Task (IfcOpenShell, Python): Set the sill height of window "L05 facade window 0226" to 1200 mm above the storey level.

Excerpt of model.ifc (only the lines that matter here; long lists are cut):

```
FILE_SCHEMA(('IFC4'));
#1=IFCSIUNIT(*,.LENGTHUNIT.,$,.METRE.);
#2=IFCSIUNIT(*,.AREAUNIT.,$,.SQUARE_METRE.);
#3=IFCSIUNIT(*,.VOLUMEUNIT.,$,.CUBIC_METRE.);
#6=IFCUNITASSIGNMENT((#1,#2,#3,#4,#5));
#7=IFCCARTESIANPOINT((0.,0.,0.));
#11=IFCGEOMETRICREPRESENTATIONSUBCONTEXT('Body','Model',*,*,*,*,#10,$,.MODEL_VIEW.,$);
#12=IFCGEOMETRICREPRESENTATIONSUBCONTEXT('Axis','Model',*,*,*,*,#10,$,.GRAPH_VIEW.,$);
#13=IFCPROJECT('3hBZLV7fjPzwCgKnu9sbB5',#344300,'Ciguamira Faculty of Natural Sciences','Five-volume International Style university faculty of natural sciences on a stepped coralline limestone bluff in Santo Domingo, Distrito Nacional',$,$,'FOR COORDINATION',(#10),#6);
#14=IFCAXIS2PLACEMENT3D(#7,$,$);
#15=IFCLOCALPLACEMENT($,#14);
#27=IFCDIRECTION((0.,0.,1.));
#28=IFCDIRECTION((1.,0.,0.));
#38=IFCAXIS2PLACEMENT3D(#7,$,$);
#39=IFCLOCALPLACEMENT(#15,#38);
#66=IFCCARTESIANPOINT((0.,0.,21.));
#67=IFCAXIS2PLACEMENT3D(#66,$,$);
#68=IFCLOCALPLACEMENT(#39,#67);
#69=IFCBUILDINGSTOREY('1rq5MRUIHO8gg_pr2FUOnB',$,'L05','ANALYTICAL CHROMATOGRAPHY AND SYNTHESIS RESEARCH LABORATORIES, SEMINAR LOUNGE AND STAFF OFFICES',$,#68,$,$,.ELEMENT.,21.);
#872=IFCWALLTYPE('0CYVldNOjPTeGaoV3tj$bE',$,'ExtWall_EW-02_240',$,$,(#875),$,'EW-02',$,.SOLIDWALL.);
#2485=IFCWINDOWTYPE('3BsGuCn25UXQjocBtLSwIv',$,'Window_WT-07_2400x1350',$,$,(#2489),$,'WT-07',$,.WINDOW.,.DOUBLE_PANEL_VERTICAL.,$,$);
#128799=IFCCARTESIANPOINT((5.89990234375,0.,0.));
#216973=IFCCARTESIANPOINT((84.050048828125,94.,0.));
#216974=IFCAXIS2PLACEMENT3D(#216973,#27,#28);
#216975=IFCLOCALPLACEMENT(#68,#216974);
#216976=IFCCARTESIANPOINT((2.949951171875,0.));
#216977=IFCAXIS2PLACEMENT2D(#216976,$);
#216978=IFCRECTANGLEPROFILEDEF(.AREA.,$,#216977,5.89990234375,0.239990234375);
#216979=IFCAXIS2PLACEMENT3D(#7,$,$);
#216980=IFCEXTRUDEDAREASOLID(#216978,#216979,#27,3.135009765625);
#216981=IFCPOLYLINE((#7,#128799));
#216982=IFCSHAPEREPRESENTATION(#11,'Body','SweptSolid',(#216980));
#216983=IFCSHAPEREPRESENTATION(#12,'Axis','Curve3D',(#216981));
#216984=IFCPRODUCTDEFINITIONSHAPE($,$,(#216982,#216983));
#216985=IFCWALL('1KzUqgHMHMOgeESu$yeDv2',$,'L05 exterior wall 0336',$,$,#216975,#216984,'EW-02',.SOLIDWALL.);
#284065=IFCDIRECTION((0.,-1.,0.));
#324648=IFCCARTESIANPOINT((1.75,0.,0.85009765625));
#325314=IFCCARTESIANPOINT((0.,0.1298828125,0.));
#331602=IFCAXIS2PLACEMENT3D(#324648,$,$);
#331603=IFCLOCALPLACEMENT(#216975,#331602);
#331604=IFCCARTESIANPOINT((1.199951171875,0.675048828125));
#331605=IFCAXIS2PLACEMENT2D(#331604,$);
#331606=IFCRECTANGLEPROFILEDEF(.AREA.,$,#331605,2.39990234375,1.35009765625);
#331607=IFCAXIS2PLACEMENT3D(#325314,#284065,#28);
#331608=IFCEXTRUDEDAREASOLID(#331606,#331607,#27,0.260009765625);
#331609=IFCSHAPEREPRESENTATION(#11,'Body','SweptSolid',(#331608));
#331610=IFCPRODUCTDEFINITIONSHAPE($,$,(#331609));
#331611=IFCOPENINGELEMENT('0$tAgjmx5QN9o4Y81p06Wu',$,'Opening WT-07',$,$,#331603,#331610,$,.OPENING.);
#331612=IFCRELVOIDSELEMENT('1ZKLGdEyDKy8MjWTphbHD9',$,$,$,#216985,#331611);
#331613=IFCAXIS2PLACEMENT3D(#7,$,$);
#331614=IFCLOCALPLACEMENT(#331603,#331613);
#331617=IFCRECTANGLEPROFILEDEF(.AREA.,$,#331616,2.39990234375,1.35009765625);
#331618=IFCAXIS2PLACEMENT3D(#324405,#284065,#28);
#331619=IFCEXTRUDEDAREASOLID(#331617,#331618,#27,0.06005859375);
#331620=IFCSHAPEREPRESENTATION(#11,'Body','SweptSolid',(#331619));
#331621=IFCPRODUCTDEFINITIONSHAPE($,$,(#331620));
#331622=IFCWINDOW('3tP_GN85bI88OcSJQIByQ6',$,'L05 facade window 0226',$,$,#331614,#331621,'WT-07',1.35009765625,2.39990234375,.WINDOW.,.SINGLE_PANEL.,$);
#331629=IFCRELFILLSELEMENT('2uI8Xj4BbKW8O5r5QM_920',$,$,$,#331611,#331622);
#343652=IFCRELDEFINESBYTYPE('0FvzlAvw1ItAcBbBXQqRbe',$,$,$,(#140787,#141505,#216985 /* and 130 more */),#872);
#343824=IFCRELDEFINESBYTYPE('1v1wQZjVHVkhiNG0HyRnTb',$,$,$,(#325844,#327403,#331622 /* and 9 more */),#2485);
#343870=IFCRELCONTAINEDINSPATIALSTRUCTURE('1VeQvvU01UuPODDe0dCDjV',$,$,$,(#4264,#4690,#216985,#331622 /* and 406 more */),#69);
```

```python
import numpy as np
import ifcopenshell
import ifcopenshell.api.geometry
import ifcopenshell.geom
import ifcopenshell.util.element
import ifcopenshell.util.placement
import ifcopenshell.util.shape
import ifcopenshell.util.unit

model = ifcopenshell.open("model.ifc")
unit_scale = ifcopenshell.util.unit.calculate_unit_scale(model)

window = model.by_guid("3tP_GN85bI88OcSJQIByQ6")
opening = window.FillsVoids[0].RelatingOpeningElement
storey = ifcopenshell.util.element.get_container(window, ifc_class="IfcBuildingStorey")
level = ifcopenshell.util.placement.get_local_placement(storey.ObjectPlacement)[2, 3]

# The opening's origin need not be at the sill, so measure its lowest point.
shape = ifcopenshell.geom.create_shape(ifcopenshell.geom.settings(), opening)
bottom = ifcopenshell.util.shape.get_shape_bottom_elevation(shape, shape.geometry) / unit_scale
dz = level + 1.2 / unit_scale - bottom

shift = np.array([0.0, 0.0, dz])
# The window is placed relative to its opening, so it follows when the opening moves.
matrix = ifcopenshell.util.placement.get_local_placement(opening.ObjectPlacement)
matrix[:3, 3] += shift
ifcopenshell.api.geometry.edit_object_placement(
    model, product=opening, matrix=matrix, is_si=False, should_transform_children=True
)

print(f"moved by {dz * unit_scale:+.3f} m")

model.write("model-out.ifc")
```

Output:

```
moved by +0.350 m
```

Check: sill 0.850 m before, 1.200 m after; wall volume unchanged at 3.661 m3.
